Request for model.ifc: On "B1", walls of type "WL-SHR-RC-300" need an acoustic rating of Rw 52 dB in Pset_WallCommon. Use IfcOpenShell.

First a look at what the model holds.

```python
import ifcopenshell
import ifcopenshell.util.element

model = ifcopenshell.open("model.ifc")
print(model.schema)
storey = next(s for s in model.by_type("IfcBuildingStorey") if s.Name == "B1")
walls = [e for e in ifcopenshell.util.element.get_decomposition(storey) if e.is_a("IfcWall")]
seen = {}
for e in walls:
    element_type = ifcopenshell.util.element.get_type(e)
    key = (element_type.Name if element_type != e and element_type else None, ifcopenshell.util.element.get_pset(e, "Pset_WallCommon", "AcousticRating"))
    seen[key] = seen.get(key, 0) + 1
for (name, value), count in sorted(seen.items(), key=str):
    print(count, "x", name, "|", value)
```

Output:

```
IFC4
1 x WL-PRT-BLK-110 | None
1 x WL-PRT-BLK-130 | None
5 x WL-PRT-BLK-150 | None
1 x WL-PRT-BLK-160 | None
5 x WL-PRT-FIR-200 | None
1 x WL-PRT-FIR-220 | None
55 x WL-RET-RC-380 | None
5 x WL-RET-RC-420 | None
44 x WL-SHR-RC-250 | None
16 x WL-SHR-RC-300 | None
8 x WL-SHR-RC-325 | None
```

```python
import ifcopenshell
import ifcopenshell.api.pset
import ifcopenshell.util.element

model = ifcopenshell.open("model.ifc")

storey = next(s for s in model.by_type("IfcBuildingStorey") if s.Name == "B1")
walls = [e for e in ifcopenshell.util.element.get_decomposition(storey) if e.is_a("IfcWall")]

count = 0
for e in walls:
    element_type = ifcopenshell.util.element.get_type(e)
    if element_type in (None, e) or element_type.Name != "WL-SHR-RC-300":
        continue
    # add_pset returns the element's existing set when there is one.
    pset = ifcopenshell.api.pset.add_pset(model, product=e, name="Pset_WallCommon")
    ifcopenshell.api.pset.edit_pset(model, pset=pset, properties={"AcousticRating": "Rw 52 dB"})
    count += 1

print(count, "walls updated")

model.write("model_rev.ifc")
```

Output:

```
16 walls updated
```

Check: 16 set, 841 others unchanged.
